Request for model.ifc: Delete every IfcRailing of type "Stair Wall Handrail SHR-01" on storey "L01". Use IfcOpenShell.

First a look at what the model holds.

```python
import ifcopenshell
import ifcopenshell.util.element

model = ifcopenshell.open("model.ifc")
print(model.schema)
storey = next(s for s in model.by_type("IfcBuildingStorey") if s.Name == "L01")
railings = [e for e in ifcopenshell.util.element.get_decomposition(storey) if e.is_a("IfcRailing")]
seen = {}
for e in railings:
    element_type = ifcopenshell.util.element.get_type(e)
    name = element_type.Name if element_type not in (None, e) else None
    seen[name] = seen.get(name, 0) + 1
for name, count in sorted(seen.items(), key=str):
    print(count, "x", name)
```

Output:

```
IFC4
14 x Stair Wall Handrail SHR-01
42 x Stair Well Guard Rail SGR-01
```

```python
import ifcopenshell
import ifcopenshell.api.root
import ifcopenshell.util.element

model = ifcopenshell.open("model.ifc")

storey = next(s for s in model.by_type("IfcBuildingStorey") if s.Name == "L01")
railings = [e for e in ifcopenshell.util.element.get_decomposition(storey) if e.is_a("IfcRailing")]
targets = [e for e in railings if (t := ifcopenshell.util.element.get_type(e)) not in (None, e) and t.Name == "Stair Wall Handrail SHR-01"]

for e in targets:
    ifcopenshell.api.root.remove_product(model, product=e)
print(len(targets), "removed")

model.write("model_v2.ifc")
```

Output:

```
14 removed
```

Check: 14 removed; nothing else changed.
